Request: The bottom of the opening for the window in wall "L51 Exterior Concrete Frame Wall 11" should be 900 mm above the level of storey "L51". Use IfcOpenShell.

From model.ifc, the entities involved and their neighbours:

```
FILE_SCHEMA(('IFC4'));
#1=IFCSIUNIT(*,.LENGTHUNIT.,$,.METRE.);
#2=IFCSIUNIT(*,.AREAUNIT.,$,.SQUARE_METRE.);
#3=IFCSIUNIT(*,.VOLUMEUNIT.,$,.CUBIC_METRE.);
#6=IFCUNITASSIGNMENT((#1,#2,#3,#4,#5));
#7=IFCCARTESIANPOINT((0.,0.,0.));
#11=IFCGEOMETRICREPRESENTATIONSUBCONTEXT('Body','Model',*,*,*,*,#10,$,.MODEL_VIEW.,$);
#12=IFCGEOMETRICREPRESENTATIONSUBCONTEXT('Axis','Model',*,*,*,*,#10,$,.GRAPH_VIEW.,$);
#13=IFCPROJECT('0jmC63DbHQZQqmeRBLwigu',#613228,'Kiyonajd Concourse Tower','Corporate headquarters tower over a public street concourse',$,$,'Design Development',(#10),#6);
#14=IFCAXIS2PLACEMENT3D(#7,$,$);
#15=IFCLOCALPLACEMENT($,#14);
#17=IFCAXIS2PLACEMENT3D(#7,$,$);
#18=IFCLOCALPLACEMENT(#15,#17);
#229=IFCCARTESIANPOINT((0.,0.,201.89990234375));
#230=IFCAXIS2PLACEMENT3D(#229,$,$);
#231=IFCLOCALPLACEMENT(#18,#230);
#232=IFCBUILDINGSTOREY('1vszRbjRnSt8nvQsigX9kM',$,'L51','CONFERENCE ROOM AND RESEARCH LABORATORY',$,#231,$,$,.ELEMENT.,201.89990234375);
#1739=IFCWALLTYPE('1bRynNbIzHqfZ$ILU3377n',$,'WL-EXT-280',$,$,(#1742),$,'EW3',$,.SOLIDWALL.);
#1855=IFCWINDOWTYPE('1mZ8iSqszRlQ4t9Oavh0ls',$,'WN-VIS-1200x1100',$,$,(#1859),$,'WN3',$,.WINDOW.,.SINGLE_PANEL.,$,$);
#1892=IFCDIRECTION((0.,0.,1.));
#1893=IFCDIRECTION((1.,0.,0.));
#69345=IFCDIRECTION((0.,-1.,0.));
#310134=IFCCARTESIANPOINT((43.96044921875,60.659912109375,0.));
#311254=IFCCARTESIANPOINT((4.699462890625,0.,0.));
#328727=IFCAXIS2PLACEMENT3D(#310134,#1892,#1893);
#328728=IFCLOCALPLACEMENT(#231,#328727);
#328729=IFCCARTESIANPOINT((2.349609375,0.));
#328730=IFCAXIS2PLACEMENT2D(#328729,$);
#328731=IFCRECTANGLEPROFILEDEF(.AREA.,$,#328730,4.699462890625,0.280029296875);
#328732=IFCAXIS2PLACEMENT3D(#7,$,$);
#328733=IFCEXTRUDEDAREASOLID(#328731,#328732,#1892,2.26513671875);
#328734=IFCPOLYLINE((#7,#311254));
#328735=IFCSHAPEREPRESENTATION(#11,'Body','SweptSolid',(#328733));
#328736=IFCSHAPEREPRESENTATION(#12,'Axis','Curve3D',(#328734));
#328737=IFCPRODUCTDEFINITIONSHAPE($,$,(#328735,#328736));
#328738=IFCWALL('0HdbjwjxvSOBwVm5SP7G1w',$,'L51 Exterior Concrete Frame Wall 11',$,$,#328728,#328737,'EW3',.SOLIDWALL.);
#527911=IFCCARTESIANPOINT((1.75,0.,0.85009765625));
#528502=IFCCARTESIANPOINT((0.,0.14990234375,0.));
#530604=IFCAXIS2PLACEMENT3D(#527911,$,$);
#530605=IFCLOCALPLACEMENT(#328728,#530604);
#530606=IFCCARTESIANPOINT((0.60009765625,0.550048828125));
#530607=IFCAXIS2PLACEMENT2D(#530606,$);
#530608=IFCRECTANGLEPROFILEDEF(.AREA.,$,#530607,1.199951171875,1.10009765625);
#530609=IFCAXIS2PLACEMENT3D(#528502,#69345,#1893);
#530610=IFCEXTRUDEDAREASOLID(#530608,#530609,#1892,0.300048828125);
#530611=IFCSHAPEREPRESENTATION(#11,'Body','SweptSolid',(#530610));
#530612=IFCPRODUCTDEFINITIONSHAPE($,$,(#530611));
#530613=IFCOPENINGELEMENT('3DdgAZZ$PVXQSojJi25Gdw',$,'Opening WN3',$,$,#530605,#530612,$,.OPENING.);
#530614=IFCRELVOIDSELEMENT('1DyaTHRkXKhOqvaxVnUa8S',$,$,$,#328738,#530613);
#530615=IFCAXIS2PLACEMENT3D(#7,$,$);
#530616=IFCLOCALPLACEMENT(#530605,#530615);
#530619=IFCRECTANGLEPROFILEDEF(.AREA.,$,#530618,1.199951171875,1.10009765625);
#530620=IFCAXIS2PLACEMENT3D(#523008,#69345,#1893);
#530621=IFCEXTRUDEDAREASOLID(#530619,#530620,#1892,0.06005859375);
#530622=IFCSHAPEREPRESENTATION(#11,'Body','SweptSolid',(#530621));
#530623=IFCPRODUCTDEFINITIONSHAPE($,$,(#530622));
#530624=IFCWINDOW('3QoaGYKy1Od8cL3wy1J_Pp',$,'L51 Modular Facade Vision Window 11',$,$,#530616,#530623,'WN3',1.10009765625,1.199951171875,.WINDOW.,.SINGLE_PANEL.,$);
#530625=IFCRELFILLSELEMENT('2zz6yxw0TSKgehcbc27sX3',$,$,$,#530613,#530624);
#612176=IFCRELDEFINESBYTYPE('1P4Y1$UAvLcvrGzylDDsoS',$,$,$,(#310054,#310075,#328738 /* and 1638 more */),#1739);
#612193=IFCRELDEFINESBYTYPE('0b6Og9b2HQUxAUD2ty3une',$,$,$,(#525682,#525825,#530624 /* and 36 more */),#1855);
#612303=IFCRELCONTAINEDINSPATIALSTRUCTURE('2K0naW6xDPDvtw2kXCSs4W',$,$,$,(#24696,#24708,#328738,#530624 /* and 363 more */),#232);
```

```python
import numpy as np
import ifcopenshell
import ifcopenshell.api.geometry
import ifcopenshell.geom
import ifcopenshell.util.element
import ifcopenshell.util.placement
import ifcopenshell.util.shape
import ifcopenshell.util.unit

model = ifcopenshell.open("model.ifc")
unit_scale = ifcopenshell.util.unit.calculate_unit_scale(model)

window = model.by_guid("3QoaGYKy1Od8cL3wy1J_Pp")
opening = window.FillsVoids[0].RelatingOpeningElement
storey = ifcopenshell.util.element.get_container(window, ifc_class="IfcBuildingStorey")
level = ifcopenshell.util.placement.get_local_placement(storey.ObjectPlacement)[2, 3]

# The opening's origin need not be at the sill, so measure its lowest point.
shape = ifcopenshell.geom.create_shape(ifcopenshell.geom.settings(), opening)
bottom = ifcopenshell.util.shape.get_shape_bottom_elevation(shape, shape.geometry) / unit_scale
dz = level + 0.9 / unit_scale - bottom

shift = np.array([0.0, 0.0, dz])
# The window is placed relative to its opening, so it follows when the opening moves.
matrix = ifcopenshell.util.placement.get_local_placement(opening.ObjectPlacement)
matrix[:3, 3] += shift
ifcopenshell.api.geometry.edit_object_placement(
    model, product=opening, matrix=matrix, is_si=False, should_transform_children=True
)

print(f"moved by {dz * unit_scale:+.3f} m")

model.write("model_updated.ifc")
```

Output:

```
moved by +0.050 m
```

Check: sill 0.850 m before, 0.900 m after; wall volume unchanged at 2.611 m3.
